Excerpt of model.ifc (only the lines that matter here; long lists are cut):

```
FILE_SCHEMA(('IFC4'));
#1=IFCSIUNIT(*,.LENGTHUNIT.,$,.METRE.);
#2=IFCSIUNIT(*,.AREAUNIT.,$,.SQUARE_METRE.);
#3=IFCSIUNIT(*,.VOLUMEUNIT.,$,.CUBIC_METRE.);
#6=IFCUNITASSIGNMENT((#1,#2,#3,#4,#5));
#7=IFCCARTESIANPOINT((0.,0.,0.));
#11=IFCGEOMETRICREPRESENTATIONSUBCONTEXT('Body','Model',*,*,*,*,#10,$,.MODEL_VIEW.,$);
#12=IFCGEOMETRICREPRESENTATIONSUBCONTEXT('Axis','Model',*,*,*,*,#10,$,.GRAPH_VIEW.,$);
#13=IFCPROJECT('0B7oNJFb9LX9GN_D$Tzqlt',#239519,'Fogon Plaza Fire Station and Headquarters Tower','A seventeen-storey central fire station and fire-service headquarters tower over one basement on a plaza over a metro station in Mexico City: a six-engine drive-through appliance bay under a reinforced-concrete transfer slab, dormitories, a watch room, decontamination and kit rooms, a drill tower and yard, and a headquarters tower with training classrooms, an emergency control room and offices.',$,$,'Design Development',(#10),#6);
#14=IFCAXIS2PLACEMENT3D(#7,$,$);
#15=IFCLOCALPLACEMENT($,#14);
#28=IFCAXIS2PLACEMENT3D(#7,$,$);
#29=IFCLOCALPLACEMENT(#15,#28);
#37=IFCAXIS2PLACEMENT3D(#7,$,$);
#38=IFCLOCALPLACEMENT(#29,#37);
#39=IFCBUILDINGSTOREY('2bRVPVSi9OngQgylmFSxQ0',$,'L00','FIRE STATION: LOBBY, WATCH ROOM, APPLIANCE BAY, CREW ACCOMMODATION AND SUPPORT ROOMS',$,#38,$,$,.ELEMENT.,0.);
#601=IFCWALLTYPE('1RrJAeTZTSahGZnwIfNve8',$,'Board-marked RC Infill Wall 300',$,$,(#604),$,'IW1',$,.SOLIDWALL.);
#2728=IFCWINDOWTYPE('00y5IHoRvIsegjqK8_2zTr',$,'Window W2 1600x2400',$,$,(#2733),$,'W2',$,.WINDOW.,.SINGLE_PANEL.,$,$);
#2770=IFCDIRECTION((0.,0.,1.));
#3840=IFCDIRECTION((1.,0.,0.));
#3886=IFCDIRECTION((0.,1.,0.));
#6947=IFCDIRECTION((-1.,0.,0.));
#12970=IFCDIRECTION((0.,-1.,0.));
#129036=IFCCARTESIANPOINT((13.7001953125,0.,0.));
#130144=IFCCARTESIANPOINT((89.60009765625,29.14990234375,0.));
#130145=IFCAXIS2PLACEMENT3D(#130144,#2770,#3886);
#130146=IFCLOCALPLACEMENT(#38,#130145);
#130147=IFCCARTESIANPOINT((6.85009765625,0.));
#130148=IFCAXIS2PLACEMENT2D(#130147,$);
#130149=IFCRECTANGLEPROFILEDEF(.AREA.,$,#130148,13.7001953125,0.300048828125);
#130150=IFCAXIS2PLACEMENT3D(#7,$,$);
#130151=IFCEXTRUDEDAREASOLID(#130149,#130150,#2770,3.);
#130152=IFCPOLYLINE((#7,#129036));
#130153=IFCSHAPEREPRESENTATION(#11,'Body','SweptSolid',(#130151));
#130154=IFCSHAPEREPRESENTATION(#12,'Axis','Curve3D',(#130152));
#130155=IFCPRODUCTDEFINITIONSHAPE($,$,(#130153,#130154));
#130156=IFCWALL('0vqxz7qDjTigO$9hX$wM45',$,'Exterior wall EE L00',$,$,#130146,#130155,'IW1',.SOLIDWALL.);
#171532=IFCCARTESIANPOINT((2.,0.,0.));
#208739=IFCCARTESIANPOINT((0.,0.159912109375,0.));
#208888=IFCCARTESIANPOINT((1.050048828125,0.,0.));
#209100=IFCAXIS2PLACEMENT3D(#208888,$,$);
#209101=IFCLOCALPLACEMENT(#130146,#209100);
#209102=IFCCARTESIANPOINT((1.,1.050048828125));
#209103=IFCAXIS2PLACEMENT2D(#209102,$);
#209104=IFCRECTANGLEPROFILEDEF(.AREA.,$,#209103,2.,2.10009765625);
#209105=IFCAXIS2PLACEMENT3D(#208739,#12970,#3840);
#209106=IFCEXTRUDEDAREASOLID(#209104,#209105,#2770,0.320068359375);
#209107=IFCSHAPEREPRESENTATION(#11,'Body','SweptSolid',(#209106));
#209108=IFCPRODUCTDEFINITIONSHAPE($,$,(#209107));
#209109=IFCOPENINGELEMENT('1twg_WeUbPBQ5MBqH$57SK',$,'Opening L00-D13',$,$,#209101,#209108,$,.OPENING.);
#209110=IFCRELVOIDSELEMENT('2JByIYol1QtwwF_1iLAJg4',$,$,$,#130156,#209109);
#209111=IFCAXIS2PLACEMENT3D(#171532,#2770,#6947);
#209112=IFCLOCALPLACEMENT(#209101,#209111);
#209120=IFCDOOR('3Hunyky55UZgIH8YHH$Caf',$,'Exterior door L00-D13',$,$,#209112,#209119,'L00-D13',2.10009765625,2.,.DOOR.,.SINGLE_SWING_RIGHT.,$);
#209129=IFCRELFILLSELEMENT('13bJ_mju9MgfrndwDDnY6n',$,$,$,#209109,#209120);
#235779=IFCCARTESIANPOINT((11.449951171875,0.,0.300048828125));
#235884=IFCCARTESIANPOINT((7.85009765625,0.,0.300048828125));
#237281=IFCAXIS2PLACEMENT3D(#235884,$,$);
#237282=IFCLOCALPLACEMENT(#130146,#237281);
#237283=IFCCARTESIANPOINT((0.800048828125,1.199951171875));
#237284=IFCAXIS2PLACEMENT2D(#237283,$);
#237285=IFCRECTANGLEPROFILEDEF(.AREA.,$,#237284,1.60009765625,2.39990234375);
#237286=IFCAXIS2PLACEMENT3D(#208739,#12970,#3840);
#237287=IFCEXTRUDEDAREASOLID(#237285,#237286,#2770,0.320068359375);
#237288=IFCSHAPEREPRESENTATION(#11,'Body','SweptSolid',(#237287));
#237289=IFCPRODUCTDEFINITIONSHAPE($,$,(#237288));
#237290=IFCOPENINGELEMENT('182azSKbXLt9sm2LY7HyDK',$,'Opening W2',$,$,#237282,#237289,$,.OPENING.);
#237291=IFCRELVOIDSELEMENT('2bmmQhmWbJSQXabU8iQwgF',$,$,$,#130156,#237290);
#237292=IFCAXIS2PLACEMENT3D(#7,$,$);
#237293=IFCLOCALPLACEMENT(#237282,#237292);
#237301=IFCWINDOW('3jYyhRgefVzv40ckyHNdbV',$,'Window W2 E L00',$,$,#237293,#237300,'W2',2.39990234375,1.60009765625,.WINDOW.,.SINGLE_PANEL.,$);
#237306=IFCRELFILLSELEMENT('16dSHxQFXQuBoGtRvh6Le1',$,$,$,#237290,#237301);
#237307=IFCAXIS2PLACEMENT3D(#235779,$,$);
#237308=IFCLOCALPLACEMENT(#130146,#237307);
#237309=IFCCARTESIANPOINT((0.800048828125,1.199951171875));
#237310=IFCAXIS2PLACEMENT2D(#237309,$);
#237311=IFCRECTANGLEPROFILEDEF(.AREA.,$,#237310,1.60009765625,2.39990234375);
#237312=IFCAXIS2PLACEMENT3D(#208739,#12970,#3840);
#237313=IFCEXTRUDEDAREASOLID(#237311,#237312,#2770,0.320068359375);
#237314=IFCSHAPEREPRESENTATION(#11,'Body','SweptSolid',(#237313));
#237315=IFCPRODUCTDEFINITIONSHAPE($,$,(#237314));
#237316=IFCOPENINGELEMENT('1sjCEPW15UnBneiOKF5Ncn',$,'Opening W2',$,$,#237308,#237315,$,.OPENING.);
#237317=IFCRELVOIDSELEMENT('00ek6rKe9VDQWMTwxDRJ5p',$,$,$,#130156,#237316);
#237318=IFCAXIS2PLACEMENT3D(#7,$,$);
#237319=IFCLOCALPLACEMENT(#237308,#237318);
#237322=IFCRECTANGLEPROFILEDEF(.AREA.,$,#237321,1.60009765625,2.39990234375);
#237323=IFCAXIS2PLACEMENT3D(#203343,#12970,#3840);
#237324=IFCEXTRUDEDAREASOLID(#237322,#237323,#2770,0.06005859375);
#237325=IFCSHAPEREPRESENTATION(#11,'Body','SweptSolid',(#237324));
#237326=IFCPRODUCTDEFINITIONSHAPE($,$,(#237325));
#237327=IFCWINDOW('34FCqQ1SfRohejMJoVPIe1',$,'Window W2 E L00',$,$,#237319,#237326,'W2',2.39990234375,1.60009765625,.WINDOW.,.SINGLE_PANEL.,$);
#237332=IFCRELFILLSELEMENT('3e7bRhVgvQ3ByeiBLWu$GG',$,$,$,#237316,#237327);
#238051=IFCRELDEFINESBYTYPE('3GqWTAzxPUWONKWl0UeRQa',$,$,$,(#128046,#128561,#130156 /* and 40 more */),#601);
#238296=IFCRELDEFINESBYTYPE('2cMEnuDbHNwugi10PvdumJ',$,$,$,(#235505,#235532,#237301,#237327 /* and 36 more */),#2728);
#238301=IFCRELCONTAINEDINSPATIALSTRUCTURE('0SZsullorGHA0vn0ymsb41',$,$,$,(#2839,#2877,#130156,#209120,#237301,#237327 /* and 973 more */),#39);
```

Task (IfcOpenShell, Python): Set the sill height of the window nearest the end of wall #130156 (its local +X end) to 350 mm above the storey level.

```python
import numpy as np
import ifcopenshell
import ifcopenshell.api.geometry
import ifcopenshell.geom
import ifcopenshell.util.element
import ifcopenshell.util.placement
import ifcopenshell.util.shape
import ifcopenshell.util.unit

model = ifcopenshell.open("model.ifc")
unit_scale = ifcopenshell.util.unit.calculate_unit_scale(model)

window = model.by_id(237327)
opening = window.FillsVoids[0].RelatingOpeningElement
storey = ifcopenshell.util.element.get_container(window, ifc_class="IfcBuildingStorey")
level = ifcopenshell.util.placement.get_local_placement(storey.ObjectPlacement)[2, 3]

# The opening's origin need not be at the sill, so measure its lowest point.
shape = ifcopenshell.geom.create_shape(ifcopenshell.geom.settings(), opening)
bottom = ifcopenshell.util.shape.get_shape_bottom_elevation(shape, shape.geometry) / unit_scale
dz = level + 0.35 / unit_scale - bottom

shift = np.array([0.0, 0.0, dz])
# The window is placed relative to its opening, so it follows when the opening moves.
matrix = ifcopenshell.util.placement.get_local_placement(opening.ObjectPlacement)
matrix[:3, 3] += shift
ifcopenshell.api.geometry.edit_object_placement(
    model, product=opening, matrix=matrix, is_si=False, should_transform_children=True
)

print(f"moved by {dz * unit_scale:+.3f} m")

model.write("model_rev.ifc")
```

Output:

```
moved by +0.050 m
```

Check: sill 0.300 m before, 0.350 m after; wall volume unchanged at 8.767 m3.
